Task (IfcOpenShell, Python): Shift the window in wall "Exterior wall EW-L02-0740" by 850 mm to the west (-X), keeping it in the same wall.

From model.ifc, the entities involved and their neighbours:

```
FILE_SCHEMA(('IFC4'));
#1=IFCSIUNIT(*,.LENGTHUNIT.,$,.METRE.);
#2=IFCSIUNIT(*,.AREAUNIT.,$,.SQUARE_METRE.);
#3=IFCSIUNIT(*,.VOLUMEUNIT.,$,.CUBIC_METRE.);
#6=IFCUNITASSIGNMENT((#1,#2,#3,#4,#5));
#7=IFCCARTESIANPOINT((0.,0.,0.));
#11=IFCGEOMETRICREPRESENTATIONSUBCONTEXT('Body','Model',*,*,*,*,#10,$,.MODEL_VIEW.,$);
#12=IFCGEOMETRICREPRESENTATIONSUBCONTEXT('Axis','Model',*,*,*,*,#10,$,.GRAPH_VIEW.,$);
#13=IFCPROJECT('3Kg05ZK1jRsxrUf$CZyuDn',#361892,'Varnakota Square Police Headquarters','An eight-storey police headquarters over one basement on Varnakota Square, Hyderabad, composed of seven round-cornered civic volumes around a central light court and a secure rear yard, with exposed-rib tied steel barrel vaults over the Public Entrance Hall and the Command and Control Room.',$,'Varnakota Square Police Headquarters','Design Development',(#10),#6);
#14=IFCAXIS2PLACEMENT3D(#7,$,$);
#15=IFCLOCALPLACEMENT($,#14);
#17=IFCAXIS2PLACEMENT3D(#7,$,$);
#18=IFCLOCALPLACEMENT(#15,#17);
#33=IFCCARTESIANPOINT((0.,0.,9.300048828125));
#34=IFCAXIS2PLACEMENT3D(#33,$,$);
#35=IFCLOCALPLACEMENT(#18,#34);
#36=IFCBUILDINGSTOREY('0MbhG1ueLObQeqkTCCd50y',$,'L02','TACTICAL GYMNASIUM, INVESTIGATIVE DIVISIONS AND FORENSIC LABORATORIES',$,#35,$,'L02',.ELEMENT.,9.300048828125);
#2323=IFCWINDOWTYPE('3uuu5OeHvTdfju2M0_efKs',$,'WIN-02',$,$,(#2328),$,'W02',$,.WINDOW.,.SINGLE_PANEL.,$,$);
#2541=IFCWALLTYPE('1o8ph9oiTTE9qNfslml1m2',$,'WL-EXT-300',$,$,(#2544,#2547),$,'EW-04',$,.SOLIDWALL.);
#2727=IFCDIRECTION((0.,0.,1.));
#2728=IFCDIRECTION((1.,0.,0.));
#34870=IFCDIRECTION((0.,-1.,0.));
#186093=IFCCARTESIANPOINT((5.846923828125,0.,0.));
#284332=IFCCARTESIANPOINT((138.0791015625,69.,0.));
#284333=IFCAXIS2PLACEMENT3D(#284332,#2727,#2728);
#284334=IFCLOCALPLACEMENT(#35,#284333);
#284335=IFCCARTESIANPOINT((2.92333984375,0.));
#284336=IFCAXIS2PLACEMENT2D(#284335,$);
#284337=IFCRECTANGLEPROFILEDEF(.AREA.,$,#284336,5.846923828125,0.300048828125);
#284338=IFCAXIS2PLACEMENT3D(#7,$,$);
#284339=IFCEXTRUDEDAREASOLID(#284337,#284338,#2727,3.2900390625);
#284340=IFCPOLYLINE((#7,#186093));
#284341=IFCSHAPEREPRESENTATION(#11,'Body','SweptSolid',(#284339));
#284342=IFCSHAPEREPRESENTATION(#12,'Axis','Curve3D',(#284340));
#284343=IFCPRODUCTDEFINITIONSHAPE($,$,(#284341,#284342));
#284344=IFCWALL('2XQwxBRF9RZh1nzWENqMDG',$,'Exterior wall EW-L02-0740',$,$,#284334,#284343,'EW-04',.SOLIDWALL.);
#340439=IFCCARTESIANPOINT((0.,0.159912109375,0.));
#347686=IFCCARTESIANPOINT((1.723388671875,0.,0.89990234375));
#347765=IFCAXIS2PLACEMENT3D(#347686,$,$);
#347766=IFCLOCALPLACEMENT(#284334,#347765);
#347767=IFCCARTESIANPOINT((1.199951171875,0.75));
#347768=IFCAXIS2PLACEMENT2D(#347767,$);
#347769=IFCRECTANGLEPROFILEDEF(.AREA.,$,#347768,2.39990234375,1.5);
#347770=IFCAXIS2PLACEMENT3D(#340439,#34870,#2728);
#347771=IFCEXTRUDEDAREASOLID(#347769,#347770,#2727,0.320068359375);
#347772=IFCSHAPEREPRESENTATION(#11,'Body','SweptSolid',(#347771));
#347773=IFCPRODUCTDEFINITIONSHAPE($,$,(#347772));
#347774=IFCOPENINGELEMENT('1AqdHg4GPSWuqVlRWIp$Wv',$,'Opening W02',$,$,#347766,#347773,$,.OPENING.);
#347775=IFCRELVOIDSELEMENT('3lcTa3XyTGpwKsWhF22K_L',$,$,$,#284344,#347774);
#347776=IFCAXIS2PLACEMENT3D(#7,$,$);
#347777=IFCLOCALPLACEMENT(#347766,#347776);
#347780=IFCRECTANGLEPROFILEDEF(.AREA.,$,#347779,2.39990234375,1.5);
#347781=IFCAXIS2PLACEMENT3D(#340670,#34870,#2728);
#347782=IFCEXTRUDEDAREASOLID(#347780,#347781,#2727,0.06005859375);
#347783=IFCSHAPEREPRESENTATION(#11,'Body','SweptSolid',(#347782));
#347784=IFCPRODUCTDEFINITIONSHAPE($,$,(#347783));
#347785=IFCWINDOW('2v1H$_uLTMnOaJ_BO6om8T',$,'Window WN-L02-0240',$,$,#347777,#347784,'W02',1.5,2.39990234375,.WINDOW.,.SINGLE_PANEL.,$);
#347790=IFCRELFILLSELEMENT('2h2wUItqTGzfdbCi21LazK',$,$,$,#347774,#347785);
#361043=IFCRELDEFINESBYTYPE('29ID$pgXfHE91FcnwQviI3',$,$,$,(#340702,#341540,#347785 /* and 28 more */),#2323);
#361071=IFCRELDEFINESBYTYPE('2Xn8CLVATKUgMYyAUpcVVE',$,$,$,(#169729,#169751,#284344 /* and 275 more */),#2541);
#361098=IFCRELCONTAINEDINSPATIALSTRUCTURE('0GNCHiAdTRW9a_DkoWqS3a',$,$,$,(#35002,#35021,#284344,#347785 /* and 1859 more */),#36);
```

```python
import ifcopenshell
import ifcopenshell.api.geometry
import ifcopenshell.util.placement
import ifcopenshell.util.unit

model = ifcopenshell.open("model.ifc")
unit_scale = ifcopenshell.util.unit.calculate_unit_scale(model)

window = model.by_guid("2v1H$_uLTMnOaJ_BO6om8T")
opening = window.FillsVoids[0].RelatingOpeningElement
wall = opening.VoidsElements[0].RelatingBuildingElement

wall_matrix = ifcopenshell.util.placement.get_local_placement(wall.ObjectPlacement)
shift = wall_matrix[:3, 0] * -0.85 / unit_scale
before = ifcopenshell.util.placement.get_local_placement(window.ObjectPlacement)[:3, 3].copy()

# The window is placed relative to its opening, so it follows when the opening moves.
matrix = ifcopenshell.util.placement.get_local_placement(opening.ObjectPlacement)
matrix[:3, 3] += shift
ifcopenshell.api.geometry.edit_object_placement(
    model, product=opening, matrix=matrix, is_si=False, should_transform_children=True
)

after = ifcopenshell.util.placement.get_local_placement(window.ObjectPlacement)[:3, 3]
print("window moved by", (after - before).round(3) + 0.0)

model.write("model_updated.ifc")
```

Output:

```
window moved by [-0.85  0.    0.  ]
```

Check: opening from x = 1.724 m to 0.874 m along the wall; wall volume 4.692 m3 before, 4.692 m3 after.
